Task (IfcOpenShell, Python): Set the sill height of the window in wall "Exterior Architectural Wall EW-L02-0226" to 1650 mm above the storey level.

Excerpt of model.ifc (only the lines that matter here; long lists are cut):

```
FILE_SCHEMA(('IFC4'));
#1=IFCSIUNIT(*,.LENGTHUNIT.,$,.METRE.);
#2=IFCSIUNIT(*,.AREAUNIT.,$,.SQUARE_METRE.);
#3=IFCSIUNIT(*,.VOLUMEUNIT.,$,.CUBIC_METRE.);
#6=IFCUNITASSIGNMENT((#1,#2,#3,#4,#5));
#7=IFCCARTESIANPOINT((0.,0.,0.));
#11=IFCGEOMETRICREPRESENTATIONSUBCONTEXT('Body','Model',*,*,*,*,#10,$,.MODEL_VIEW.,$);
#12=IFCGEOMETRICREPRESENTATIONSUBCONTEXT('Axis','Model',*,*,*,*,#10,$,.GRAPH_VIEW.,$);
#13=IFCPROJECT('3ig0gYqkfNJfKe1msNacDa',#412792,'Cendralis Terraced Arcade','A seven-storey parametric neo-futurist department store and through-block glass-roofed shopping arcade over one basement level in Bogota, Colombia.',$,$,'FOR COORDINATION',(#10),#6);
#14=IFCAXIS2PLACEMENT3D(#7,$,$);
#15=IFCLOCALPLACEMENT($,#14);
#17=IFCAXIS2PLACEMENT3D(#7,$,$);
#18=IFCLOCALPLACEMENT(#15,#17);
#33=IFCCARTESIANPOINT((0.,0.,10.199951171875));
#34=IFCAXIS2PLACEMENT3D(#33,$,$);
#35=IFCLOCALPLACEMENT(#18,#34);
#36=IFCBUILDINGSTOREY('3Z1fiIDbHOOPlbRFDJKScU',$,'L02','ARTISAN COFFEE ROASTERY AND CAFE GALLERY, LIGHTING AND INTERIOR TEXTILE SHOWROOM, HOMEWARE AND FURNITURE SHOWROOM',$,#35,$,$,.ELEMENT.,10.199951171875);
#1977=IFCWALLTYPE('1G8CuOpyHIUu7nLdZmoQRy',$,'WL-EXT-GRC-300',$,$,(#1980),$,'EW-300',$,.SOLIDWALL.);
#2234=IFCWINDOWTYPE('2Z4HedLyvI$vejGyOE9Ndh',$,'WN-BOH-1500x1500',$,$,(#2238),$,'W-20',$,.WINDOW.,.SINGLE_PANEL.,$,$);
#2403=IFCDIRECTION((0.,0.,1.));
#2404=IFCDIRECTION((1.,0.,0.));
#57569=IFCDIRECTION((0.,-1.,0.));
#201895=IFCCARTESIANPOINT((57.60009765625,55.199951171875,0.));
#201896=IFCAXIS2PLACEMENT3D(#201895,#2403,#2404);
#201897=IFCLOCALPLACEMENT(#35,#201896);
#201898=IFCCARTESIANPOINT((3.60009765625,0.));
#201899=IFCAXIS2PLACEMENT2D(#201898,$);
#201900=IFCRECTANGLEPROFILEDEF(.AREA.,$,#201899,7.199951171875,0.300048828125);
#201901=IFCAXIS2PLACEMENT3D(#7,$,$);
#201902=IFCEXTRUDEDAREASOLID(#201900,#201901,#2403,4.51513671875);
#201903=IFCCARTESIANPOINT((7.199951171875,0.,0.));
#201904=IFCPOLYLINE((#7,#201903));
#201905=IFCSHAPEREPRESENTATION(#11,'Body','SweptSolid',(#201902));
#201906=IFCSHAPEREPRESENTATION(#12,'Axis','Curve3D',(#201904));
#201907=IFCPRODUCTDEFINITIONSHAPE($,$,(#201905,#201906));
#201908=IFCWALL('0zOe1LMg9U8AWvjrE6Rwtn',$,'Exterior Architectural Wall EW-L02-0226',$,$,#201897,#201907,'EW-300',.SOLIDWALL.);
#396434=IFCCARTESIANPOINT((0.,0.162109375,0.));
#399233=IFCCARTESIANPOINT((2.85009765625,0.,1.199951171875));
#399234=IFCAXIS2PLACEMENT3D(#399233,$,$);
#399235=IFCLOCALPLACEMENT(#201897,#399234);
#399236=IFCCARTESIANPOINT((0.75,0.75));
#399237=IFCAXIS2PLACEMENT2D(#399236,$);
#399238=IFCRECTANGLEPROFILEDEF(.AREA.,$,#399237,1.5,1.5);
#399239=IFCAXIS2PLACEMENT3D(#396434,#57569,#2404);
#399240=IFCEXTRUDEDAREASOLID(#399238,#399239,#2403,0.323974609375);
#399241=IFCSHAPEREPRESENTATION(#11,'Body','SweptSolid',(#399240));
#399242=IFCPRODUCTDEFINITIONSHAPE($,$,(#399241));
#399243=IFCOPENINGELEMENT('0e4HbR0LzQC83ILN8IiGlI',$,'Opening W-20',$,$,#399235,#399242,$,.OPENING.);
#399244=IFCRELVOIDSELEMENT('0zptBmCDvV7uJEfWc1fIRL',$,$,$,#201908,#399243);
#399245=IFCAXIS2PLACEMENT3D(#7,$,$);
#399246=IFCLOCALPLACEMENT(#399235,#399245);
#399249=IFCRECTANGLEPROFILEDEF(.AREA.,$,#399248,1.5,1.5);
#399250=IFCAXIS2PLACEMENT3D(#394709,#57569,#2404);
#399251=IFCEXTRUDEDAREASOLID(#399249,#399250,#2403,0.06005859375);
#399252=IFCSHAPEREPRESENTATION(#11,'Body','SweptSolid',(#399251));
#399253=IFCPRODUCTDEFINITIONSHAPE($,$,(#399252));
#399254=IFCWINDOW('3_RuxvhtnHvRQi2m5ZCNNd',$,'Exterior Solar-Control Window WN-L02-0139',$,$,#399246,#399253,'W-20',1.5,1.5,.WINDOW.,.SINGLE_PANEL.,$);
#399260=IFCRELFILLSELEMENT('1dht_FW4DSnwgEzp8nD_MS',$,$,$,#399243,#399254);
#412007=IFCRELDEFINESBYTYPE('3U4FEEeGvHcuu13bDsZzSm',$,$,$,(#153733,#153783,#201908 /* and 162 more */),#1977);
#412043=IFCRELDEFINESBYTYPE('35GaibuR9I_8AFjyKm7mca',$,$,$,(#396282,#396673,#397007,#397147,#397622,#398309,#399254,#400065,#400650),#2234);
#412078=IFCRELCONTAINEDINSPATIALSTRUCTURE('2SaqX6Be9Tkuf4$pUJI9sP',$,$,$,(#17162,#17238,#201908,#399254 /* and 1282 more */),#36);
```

```python
import numpy as np
import ifcopenshell
import ifcopenshell.api.geometry
import ifcopenshell.geom
import ifcopenshell.util.element
import ifcopenshell.util.placement
import ifcopenshell.util.shape
import ifcopenshell.util.unit

model = ifcopenshell.open("model.ifc")
unit_scale = ifcopenshell.util.unit.calculate_unit_scale(model)

window = model.by_guid("3_RuxvhtnHvRQi2m5ZCNNd")
opening = window.FillsVoids[0].RelatingOpeningElement
storey = ifcopenshell.util.element.get_container(window, ifc_class="IfcBuildingStorey")
level = ifcopenshell.util.placement.get_local_placement(storey.ObjectPlacement)[2, 3]

# The opening's origin need not be at the sill, so measure its lowest point.
shape = ifcopenshell.geom.create_shape(ifcopenshell.geom.settings(), opening)
bottom = ifcopenshell.util.shape.get_shape_bottom_elevation(shape, shape.geometry) / unit_scale
dz = level + 1.65 / unit_scale - bottom

shift = np.array([0.0, 0.0, dz])
# The window is placed relative to its opening, so it follows when the opening moves.
matrix = ifcopenshell.util.placement.get_local_placement(opening.ObjectPlacement)
matrix[:3, 3] += shift
ifcopenshell.api.geometry.edit_object_placement(
    model, product=opening, matrix=matrix, is_si=False, should_transform_children=True
)

print(f"moved by {dz * unit_scale:+.3f} m")

model.write("model-out.ifc")
```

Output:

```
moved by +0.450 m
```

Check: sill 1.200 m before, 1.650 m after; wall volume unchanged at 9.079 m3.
